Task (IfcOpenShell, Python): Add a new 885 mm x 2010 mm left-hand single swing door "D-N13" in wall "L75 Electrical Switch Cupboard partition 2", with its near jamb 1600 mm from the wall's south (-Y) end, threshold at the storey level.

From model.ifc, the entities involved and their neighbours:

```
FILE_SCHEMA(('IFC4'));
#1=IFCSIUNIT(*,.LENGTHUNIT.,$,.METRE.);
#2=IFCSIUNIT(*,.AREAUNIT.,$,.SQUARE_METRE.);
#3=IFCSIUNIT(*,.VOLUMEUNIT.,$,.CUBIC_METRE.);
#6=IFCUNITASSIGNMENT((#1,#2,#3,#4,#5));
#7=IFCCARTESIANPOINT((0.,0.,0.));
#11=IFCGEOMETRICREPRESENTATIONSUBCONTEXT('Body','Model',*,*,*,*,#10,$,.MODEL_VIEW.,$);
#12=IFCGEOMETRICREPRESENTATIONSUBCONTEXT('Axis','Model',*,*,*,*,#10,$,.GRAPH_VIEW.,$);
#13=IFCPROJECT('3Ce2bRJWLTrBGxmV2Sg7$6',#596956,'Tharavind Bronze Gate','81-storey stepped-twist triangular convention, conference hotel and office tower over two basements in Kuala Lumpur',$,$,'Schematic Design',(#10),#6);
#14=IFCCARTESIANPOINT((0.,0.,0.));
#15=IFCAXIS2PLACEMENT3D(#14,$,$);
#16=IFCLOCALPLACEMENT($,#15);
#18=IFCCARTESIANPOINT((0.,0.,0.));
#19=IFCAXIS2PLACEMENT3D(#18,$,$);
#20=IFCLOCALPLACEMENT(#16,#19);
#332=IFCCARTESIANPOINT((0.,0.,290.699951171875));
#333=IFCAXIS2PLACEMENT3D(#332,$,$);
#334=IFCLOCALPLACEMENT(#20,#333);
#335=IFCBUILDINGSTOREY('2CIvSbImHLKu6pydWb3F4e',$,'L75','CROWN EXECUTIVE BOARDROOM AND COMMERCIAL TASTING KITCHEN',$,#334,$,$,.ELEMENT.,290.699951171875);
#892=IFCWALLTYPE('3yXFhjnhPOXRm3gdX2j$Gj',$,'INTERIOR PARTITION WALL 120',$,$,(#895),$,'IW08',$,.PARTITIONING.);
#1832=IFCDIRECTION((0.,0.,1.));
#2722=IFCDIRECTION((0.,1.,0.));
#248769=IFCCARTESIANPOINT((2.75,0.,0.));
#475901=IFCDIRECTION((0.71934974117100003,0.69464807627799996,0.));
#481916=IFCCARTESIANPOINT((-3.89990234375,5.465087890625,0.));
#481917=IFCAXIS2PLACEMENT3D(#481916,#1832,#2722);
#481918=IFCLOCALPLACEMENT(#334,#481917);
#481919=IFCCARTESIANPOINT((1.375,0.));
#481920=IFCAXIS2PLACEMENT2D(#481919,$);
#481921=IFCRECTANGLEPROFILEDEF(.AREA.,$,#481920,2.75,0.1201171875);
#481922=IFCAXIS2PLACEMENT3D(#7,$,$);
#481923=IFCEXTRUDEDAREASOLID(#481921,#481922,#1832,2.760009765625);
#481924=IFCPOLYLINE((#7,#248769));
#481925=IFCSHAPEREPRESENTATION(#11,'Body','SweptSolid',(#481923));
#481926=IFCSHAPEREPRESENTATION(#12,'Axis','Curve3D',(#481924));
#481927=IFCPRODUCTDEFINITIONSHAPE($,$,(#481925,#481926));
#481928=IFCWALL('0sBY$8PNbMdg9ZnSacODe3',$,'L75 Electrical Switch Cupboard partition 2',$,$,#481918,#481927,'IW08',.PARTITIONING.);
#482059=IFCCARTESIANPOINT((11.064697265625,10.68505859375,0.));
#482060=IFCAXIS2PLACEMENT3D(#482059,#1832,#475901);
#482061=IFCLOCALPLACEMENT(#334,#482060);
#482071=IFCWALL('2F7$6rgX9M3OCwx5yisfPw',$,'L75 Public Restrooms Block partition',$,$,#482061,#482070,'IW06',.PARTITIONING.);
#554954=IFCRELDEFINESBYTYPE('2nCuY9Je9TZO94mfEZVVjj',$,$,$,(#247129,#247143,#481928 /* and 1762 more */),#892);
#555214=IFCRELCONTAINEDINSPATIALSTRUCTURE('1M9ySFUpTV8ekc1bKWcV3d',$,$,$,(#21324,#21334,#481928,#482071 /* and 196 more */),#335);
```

```python
import numpy as np
import ifcopenshell
import ifcopenshell.api.feature
import ifcopenshell.api.geometry
import ifcopenshell.api.root
import ifcopenshell.api.spatial
import ifcopenshell.geom
import ifcopenshell.util.element
import ifcopenshell.util.placement
import ifcopenshell.util.representation
import ifcopenshell.util.shape
import ifcopenshell.util.unit

model = ifcopenshell.open("model.ifc")
unit_scale = ifcopenshell.util.unit.calculate_unit_scale(model)
settings = ifcopenshell.geom.settings()


def volume(element):
    """Net volume in cubic metres, openings subtracted."""
    shape = ifcopenshell.geom.create_shape(settings, element)
    return ifcopenshell.util.shape.get_volume(shape.geometry)


wall = model.by_guid("0sBY$8PNbMdg9ZnSacODe3")
storey = ifcopenshell.util.element.get_container(wall, ifc_class="IfcBuildingStorey")
context = ifcopenshell.util.representation.get_context(model, "Model", "Body", "MODEL_VIEW")
before = volume(wall)

width, height, from_end, sill = 0.885, 2.01, 1.6, 0.0  # metres

# The wall runs along its own X axis, and the end named is its -X end.
wall_shape = ifcopenshell.geom.create_shape(settings, wall)
x, y, z = ifcopenshell.util.shape.get_vertices(wall_shape.geometry).T
start = x.min() + from_end
face, thickness = float(y.min()), float(y.max() - y.min())
wall_matrix = ifcopenshell.util.placement.get_local_placement(wall.ObjectPlacement)
level = ifcopenshell.util.placement.get_local_placement(storey.ObjectPlacement)[2, 3]


def in_wall(x, y):
    """Placement at x, y metres in the wall's axes, at sill height."""
    matrix = wall_matrix.copy()
    matrix[:, 3] = wall_matrix @ np.array([x / unit_scale, y / unit_scale, 0.0, 1.0])
    matrix[2, 3] = level + sill / unit_scale
    return matrix


# Opening: a box that overshoots both wall faces by 50 mm.
opening = ifcopenshell.api.root.create_entity(model, ifc_class="IfcOpeningElement", predefined_type="OPENING")
box = ifcopenshell.api.geometry.add_wall_representation(
    model, context=context, length=width, height=height, thickness=thickness + 0.1
)
ifcopenshell.api.geometry.assign_representation(model, product=opening, representation=box)
ifcopenshell.api.geometry.edit_object_placement(model, product=opening, matrix=in_wall(start, face - 0.05), is_si=False)
ifcopenshell.api.feature.add_feature(model, feature=opening, element=wall)

door = ifcopenshell.api.root.create_entity(model, ifc_class="IfcDoor", name="D-N13", predefined_type="DOOR")
door.OverallWidth, door.OverallHeight = width / unit_scale, height / unit_scale
door.OperationType = "SINGLE_SWING_LEFT"
body = ifcopenshell.api.geometry.add_door_representation(
    model,
    context=context,
    overall_width=door.OverallWidth,
    overall_height=door.OverallHeight,
    operation_type="SINGLE_SWING_LEFT",
    lining_properties={"LiningDepth": thickness / unit_scale, "ThresholdDepth": thickness / unit_scale},
)
ifcopenshell.api.geometry.assign_representation(model, product=door, representation=body)
ifcopenshell.api.spatial.assign_container(model, products=[door], relating_structure=storey)
ifcopenshell.api.feature.add_filling(model, opening=opening, element=door)

# The lining spans the wall, so the door starts at the wall face.
ifcopenshell.api.geometry.edit_object_placement(model, product=door, matrix=in_wall(start, face), is_si=False)

after = volume(wall)

print(f"wall volume {before:.3f} -> {after:.3f} m3")

model.write("model_updated.ifc")
```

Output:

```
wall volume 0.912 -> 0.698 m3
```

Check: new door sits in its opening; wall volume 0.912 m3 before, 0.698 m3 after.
